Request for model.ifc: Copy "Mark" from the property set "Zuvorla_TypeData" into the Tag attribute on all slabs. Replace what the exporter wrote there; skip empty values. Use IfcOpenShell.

First a look at what the model holds.

```python
import ifcopenshell
import ifcopenshell.util.element

model = ifcopenshell.open("model.ifc")
print(model.schema)
slabs = model.by_type("IfcSlab")
print(len(slabs), "slabs")
for e in slabs[:8]:
    source = ifcopenshell.util.element.get_pset(e, "Zuvorla_TypeData", "Mark")
    target = e.Tag
    print(e.id(), repr(source), repr(target), sep=" | ")
```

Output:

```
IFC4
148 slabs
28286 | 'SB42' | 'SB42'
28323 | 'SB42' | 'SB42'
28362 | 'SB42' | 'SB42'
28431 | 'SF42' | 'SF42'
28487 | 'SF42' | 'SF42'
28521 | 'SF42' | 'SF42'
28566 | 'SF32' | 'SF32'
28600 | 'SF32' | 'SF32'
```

```python
import ifcopenshell
import ifcopenshell.util.element

model = ifcopenshell.open("model.ifc")

count = 0
for e in model.by_type("IfcSlab"):
    value = ifcopenshell.util.element.get_pset(e, "Zuvorla_TypeData", "Mark")
    current = e.Tag
    if not value or not value.strip() or current == value:
        continue
    e.Tag = value
    count += 1

print(count, "slabs updated")

model.write("model_v2.ifc")
```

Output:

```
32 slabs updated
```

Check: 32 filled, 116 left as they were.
